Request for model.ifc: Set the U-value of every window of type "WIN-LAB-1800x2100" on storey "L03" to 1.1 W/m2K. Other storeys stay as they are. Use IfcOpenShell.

First a look at what the model holds.

```python
import ifcopenshell
import ifcopenshell.util.element

model = ifcopenshell.open("model.ifc")
print(model.schema)
storey = next(s for s in model.by_type("IfcBuildingStorey") if s.Name == "L03")
windows = [e for e in ifcopenshell.util.element.get_decomposition(storey) if e.is_a("IfcWindow")]
seen = {}
for e in windows:
    element_type = ifcopenshell.util.element.get_type(e)
    key = (element_type.Name if element_type != e and element_type else None, ifcopenshell.util.element.get_pset(e, "Pset_WindowCommon", "ThermalTransmittance"))
    seen[key] = seen.get(key, 0) + 1
for (name, value), count in sorted(seen.items(), key=str):
    print(count, "x", name, "|", value)
```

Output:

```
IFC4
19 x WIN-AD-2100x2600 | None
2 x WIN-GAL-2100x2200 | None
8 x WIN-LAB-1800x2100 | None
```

```python
import ifcopenshell
import ifcopenshell.api.pset
import ifcopenshell.util.element

model = ifcopenshell.open("model.ifc")

storey = next(s for s in model.by_type("IfcBuildingStorey") if s.Name == "L03")
windows = [e for e in ifcopenshell.util.element.get_decomposition(storey) if e.is_a("IfcWindow")]

count = 0
for e in windows:
    element_type = ifcopenshell.util.element.get_type(e)
    if element_type in (None, e) or element_type.Name != "WIN-LAB-1800x2100":
        continue
    # add_pset returns the element's existing set when there is one.
    pset = ifcopenshell.api.pset.add_pset(model, product=e, name="Pset_WindowCommon")
    ifcopenshell.api.pset.edit_pset(model, pset=pset, properties={"ThermalTransmittance": 1.1})
    count += 1

print(count, "windows updated")

model.write("model_updated.ifc")
```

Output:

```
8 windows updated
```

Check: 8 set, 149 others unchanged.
